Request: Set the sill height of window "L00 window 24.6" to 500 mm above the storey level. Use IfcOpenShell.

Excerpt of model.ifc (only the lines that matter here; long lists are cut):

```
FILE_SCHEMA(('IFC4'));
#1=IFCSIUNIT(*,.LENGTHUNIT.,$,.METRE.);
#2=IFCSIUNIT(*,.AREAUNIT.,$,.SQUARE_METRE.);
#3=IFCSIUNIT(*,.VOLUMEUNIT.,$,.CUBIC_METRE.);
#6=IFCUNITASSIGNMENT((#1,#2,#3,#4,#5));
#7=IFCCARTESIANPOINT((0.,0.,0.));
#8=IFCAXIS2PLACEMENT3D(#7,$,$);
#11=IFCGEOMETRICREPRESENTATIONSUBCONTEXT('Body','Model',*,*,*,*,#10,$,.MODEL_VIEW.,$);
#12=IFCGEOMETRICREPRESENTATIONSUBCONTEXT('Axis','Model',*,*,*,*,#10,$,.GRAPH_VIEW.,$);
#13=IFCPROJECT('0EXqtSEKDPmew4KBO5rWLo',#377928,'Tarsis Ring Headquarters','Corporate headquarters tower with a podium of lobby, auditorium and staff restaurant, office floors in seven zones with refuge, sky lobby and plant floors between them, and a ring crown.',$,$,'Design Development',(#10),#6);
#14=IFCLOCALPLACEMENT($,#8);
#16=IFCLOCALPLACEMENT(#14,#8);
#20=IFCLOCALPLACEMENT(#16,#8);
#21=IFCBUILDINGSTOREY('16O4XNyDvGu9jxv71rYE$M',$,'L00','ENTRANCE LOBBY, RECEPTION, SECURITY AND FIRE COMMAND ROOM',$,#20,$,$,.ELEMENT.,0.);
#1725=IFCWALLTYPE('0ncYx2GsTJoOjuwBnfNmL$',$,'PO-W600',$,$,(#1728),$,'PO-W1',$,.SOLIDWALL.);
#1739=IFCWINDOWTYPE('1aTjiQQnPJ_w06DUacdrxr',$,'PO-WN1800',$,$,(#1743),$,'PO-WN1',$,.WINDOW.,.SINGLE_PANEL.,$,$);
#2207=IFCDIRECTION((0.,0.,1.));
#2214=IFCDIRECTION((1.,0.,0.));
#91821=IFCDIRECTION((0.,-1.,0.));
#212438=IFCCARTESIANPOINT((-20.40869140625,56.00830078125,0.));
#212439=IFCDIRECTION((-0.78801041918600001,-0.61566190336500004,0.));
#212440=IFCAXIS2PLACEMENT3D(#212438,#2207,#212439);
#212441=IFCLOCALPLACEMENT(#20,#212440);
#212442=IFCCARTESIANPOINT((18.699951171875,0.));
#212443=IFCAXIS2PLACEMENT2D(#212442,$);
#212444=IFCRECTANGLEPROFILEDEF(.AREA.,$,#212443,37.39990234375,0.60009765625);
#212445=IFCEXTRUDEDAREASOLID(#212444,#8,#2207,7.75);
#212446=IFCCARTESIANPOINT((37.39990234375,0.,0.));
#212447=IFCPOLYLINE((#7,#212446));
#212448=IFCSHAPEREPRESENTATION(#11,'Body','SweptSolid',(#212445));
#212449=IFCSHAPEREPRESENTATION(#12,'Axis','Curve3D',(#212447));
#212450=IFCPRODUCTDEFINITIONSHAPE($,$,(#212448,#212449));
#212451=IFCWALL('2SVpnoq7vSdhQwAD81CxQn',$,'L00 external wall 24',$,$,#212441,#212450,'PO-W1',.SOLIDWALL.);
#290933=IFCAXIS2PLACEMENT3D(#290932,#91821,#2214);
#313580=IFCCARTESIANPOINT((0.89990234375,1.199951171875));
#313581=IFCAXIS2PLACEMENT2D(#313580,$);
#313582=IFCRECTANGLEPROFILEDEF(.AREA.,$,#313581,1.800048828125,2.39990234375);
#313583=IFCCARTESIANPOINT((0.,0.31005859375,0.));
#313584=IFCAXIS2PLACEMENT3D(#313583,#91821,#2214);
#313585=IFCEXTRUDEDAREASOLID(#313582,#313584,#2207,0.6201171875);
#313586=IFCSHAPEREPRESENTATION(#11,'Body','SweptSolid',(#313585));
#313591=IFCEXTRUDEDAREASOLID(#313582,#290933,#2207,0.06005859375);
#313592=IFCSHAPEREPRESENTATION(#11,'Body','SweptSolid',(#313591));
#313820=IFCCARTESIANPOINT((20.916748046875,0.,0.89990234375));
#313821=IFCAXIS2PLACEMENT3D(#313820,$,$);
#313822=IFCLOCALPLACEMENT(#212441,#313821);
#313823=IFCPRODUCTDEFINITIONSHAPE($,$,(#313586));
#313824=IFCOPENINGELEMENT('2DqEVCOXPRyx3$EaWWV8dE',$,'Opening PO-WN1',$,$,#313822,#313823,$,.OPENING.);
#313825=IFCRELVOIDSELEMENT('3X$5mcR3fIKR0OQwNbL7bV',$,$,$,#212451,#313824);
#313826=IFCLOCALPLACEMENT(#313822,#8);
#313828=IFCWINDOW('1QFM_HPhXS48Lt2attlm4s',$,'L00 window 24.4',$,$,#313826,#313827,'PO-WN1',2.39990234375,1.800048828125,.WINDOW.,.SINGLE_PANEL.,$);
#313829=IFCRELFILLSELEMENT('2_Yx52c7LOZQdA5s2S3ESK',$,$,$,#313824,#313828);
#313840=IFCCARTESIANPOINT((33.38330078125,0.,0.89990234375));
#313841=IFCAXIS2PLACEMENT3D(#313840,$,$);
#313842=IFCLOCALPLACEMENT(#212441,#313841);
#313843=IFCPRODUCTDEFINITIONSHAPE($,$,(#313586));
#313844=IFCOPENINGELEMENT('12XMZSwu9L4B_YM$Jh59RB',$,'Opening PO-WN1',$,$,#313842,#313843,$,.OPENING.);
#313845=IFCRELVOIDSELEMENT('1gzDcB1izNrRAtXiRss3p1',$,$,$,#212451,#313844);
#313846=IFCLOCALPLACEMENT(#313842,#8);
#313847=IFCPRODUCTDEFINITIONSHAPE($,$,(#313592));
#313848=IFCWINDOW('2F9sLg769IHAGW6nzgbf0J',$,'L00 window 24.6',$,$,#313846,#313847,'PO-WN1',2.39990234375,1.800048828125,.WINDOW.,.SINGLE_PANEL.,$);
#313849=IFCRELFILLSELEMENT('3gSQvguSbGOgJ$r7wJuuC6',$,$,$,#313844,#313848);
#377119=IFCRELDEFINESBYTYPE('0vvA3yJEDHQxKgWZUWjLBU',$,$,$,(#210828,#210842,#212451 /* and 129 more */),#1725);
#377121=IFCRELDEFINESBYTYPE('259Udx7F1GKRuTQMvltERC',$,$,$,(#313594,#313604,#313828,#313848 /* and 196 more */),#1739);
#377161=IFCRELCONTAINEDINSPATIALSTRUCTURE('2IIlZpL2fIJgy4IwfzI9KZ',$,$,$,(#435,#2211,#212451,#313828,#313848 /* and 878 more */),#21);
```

```python
import numpy as np
import ifcopenshell
import ifcopenshell.api.geometry
import ifcopenshell.geom
import ifcopenshell.util.element
import ifcopenshell.util.placement
import ifcopenshell.util.shape
import ifcopenshell.util.unit

model = ifcopenshell.open("model.ifc")
unit_scale = ifcopenshell.util.unit.calculate_unit_scale(model)

window = model.by_guid("2F9sLg769IHAGW6nzgbf0J")
opening = window.FillsVoids[0].RelatingOpeningElement
storey = ifcopenshell.util.element.get_container(window, ifc_class="IfcBuildingStorey")
level = ifcopenshell.util.placement.get_local_placement(storey.ObjectPlacement)[2, 3]

# The opening's origin need not be at the sill, so measure its lowest point.
shape = ifcopenshell.geom.create_shape(ifcopenshell.geom.settings(), opening)
bottom = ifcopenshell.util.shape.get_shape_bottom_elevation(shape, shape.geometry) / unit_scale
dz = level + 0.5 / unit_scale - bottom

shift = np.array([0.0, 0.0, dz])
# The window is placed relative to its opening, so it follows when the opening moves.
matrix = ifcopenshell.util.placement.get_local_placement(opening.ObjectPlacement)
matrix[:3, 3] += shift
ifcopenshell.api.geometry.edit_object_placement(
    model, product=opening, matrix=matrix, is_si=False, should_transform_children=True
)

print(f"moved by {dz * unit_scale:+.3f} m")

model.write("model_updated.ifc")
```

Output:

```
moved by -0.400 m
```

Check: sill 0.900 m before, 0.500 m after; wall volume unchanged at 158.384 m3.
